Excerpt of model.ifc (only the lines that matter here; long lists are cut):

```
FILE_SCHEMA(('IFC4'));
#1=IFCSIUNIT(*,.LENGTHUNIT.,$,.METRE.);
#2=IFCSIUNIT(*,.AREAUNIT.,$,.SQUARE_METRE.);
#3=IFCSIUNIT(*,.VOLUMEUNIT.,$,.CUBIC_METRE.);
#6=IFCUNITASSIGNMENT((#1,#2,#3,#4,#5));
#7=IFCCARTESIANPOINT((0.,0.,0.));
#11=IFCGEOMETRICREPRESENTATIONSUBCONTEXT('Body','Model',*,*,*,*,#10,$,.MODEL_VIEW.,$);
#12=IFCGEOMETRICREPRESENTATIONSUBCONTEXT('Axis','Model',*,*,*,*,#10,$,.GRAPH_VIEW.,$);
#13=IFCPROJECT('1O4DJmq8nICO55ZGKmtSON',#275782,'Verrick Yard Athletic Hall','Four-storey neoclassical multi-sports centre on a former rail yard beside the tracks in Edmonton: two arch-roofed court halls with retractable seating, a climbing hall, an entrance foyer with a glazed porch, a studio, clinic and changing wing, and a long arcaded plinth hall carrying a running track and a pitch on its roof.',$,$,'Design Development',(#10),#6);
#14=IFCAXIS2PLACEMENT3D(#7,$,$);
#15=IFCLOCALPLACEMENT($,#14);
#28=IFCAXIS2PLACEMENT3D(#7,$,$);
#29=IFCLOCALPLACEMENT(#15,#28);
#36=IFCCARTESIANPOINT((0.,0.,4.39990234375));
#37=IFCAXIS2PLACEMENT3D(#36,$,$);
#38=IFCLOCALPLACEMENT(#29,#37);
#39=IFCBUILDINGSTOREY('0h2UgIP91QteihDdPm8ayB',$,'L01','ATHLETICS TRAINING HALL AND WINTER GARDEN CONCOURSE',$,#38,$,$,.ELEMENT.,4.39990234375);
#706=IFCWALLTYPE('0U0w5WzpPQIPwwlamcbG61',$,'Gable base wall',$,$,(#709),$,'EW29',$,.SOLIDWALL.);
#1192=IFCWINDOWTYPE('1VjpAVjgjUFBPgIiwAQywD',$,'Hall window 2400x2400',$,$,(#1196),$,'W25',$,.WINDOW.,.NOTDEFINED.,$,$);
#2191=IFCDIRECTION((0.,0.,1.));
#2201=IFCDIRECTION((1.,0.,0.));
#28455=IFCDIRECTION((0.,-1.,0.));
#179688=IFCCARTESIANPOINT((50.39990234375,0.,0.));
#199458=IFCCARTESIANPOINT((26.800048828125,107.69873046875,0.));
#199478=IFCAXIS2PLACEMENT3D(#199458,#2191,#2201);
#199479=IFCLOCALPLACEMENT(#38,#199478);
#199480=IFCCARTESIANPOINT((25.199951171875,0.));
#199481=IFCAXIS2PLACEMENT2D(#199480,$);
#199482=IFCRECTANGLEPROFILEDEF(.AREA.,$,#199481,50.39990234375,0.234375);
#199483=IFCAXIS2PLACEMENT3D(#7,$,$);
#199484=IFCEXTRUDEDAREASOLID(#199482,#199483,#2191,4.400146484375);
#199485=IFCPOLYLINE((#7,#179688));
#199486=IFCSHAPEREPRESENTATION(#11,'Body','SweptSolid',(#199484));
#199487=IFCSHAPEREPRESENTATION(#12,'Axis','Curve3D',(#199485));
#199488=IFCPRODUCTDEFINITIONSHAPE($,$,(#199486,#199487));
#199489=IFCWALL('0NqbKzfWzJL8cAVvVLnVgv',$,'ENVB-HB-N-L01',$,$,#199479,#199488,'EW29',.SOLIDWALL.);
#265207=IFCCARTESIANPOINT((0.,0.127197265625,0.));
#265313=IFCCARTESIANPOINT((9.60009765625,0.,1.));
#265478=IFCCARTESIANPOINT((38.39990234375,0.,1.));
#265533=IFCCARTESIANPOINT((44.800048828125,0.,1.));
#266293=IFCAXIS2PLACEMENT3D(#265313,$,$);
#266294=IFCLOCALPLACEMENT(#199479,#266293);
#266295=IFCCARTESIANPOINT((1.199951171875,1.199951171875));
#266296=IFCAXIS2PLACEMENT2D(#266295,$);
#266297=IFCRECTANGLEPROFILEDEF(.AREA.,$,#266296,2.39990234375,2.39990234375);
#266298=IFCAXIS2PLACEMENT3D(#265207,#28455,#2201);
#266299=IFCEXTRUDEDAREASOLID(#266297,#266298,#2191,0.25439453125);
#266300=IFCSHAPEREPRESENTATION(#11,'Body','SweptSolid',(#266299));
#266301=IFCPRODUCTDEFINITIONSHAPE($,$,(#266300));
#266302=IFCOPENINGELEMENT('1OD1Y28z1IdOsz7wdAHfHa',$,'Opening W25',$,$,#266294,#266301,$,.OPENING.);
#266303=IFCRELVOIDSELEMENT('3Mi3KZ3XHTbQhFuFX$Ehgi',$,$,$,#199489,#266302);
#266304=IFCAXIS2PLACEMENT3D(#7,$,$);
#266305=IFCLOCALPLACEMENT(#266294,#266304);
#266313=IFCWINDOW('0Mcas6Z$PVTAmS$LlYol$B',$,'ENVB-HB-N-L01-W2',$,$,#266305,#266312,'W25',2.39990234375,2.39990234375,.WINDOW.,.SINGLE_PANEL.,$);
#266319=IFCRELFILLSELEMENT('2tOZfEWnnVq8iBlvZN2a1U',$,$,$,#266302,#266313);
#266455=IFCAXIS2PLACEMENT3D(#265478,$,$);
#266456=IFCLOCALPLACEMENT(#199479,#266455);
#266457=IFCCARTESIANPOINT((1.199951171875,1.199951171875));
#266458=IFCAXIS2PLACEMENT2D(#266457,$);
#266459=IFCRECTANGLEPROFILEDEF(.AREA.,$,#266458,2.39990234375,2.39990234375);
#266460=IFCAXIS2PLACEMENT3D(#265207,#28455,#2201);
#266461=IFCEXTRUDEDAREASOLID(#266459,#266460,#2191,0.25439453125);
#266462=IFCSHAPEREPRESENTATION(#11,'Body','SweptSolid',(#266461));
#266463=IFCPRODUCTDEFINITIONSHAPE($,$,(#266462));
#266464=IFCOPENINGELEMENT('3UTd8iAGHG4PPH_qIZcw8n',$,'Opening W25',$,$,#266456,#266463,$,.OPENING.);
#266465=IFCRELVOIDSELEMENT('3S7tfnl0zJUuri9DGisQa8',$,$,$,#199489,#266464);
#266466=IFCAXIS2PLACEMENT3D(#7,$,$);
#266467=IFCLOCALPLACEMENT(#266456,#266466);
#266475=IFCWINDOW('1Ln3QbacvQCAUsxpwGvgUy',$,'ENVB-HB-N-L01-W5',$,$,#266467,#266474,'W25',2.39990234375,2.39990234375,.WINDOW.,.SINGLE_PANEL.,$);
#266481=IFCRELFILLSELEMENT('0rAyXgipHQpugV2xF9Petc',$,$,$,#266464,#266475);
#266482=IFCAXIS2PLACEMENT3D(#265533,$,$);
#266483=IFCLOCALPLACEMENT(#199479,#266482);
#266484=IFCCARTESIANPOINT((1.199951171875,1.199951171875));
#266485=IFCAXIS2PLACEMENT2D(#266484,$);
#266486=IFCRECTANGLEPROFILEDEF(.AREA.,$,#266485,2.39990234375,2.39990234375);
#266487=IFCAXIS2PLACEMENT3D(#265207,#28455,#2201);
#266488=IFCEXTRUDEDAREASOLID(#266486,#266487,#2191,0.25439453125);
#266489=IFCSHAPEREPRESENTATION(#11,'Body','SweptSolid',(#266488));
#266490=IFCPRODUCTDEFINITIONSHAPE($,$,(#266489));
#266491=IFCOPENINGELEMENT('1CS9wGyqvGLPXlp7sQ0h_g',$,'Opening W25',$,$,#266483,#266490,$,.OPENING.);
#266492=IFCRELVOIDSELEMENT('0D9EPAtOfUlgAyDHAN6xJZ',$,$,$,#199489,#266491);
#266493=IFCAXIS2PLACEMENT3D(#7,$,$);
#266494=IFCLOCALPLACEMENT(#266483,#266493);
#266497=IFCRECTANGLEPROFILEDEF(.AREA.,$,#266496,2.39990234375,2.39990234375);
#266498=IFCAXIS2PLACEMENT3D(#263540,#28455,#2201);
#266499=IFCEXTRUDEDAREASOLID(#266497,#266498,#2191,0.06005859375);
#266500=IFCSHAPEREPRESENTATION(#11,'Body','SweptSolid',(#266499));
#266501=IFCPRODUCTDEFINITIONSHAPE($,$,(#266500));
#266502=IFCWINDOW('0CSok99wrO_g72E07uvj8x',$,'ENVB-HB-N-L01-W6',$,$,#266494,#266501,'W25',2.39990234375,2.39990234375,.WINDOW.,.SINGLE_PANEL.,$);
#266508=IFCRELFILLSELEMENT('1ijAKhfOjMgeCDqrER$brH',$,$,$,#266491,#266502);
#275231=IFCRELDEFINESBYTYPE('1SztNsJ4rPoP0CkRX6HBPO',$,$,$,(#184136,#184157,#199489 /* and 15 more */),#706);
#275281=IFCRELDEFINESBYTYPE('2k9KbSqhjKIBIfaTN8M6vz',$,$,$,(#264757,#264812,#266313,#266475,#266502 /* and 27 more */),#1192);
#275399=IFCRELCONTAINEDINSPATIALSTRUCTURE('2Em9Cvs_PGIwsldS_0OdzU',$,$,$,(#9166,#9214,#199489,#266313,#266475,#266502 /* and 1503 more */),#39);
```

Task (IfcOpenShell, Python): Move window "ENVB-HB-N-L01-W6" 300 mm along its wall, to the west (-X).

```python
import ifcopenshell
import ifcopenshell.api.geometry
import ifcopenshell.util.placement

model = ifcopenshell.open("model.ifc")

window = model.by_guid("0CSok99wrO_g72E07uvj8x")
opening = window.FillsVoids[0].RelatingOpeningElement
wall = opening.VoidsElements[0].RelatingBuildingElement

wall_matrix = ifcopenshell.util.placement.get_local_placement(wall.ObjectPlacement)
shift = wall_matrix[:3, 0] * -0.3
before = ifcopenshell.util.placement.get_local_placement(window.ObjectPlacement)[:3, 3].copy()

# The window is placed relative to its opening, so it follows when the opening moves.
matrix = ifcopenshell.util.placement.get_local_placement(opening.ObjectPlacement)
matrix[:3, 3] += shift
ifcopenshell.api.geometry.edit_object_placement(
    model, product=opening, matrix=matrix, is_si=False, should_transform_children=True
)

after = ifcopenshell.util.placement.get_local_placement(window.ObjectPlacement)[:3, 3]
print("window moved by", (after - before).round(3) + 0.0)

model.write("model-out.ifc")
```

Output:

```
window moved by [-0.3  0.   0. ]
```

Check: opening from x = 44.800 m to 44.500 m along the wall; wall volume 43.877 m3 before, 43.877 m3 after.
